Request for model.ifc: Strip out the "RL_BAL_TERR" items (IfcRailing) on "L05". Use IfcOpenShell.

First a look at what the model holds.

```python
import ifcopenshell
import ifcopenshell.util.element

model = ifcopenshell.open("model.ifc")
print(model.schema)
storey = next(s for s in model.by_type("IfcBuildingStorey") if s.Name == "L05")
railings = [e for e in ifcopenshell.util.element.get_decomposition(storey) if e.is_a("IfcRailing")]
seen = {}
for e in railings:
    element_type = ifcopenshell.util.element.get_type(e)
    name = element_type.Name if element_type not in (None, e) else None
    seen[name] = seen.get(name, 0) + 1
for name, count in sorted(seen.items(), key=str):
    print(count, "x", name)
```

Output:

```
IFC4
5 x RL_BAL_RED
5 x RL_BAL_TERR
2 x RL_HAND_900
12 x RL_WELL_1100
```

```python
import ifcopenshell
import ifcopenshell.api.root
import ifcopenshell.util.element

model = ifcopenshell.open("model.ifc")

storey = next(s for s in model.by_type("IfcBuildingStorey") if s.Name == "L05")
railings = [e for e in ifcopenshell.util.element.get_decomposition(storey) if e.is_a("IfcRailing")]
targets = [e for e in railings if (t := ifcopenshell.util.element.get_type(e)) not in (None, e) and t.Name == "RL_BAL_TERR"]

for e in targets:
    ifcopenshell.api.root.remove_product(model, product=e)
print(len(targets), "removed")

model.write("model_rev.ifc")
```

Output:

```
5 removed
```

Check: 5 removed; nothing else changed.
